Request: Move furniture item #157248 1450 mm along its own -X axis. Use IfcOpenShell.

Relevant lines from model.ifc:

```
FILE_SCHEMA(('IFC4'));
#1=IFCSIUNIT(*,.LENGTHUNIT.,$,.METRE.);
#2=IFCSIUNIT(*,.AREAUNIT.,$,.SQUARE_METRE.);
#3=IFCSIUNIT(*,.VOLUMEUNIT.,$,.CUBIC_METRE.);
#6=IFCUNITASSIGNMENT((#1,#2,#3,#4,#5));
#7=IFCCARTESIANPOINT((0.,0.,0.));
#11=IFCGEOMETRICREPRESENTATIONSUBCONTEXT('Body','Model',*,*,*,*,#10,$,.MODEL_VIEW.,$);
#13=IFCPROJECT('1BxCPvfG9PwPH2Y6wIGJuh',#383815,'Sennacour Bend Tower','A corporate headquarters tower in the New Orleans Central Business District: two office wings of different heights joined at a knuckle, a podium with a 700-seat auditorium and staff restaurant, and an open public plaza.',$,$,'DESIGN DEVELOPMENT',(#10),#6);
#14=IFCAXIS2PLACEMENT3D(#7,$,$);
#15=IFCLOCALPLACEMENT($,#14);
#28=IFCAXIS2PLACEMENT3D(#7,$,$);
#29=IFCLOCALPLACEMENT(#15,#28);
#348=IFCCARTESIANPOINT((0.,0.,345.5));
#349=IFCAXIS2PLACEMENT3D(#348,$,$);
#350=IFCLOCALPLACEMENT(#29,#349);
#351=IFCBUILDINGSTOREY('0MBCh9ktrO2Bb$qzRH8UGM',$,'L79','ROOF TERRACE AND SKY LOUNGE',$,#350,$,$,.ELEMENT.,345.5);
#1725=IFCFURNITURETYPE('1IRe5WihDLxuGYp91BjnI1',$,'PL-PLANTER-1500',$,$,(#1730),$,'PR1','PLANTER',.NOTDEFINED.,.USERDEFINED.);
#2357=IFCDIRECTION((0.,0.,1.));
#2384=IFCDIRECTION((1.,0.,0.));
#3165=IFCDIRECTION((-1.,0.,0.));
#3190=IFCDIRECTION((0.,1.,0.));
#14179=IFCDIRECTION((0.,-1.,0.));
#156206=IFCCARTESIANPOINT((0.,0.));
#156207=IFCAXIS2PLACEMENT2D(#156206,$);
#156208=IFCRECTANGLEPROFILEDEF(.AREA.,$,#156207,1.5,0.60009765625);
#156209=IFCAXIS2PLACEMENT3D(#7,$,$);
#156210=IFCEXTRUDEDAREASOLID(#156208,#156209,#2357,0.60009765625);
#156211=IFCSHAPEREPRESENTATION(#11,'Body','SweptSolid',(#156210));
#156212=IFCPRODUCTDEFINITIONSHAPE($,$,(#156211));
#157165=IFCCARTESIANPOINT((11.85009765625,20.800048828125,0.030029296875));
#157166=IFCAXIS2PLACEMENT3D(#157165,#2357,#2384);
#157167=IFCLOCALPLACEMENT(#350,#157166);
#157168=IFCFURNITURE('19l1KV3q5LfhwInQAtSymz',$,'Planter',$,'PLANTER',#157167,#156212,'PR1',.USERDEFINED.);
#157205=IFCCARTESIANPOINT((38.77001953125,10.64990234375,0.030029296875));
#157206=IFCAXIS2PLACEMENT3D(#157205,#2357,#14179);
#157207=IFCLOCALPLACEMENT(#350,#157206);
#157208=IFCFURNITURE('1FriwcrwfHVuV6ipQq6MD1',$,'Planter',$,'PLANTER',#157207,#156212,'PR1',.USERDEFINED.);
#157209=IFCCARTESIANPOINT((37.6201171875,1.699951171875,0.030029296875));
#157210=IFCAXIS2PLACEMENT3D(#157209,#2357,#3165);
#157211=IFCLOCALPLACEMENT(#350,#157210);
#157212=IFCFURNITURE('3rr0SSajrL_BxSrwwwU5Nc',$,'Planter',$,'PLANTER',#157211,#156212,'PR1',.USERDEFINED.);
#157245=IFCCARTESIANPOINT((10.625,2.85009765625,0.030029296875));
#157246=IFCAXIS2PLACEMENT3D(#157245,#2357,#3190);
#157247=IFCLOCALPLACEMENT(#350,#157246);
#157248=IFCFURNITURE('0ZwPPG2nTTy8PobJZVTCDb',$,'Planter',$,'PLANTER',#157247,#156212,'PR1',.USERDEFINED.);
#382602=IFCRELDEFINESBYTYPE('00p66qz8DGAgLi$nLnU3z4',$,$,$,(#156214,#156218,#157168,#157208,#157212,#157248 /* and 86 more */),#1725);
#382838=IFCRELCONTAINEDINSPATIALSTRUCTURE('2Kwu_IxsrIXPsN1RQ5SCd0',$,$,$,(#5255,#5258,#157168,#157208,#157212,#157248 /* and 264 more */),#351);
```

```python
import ifcopenshell
import ifcopenshell.api.geometry
import ifcopenshell.util.placement
import ifcopenshell.util.unit

model = ifcopenshell.open("model.ifc")
unit_scale = ifcopenshell.util.unit.calculate_unit_scale(model)

item = model.by_guid("0ZwPPG2nTTy8PobJZVTCDb")
matrix = ifcopenshell.util.placement.get_local_placement(item.ObjectPlacement)
matrix[:3, 3] -= matrix[:3, 0] * 1.45 / unit_scale
ifcopenshell.api.geometry.edit_object_placement(model, product=item, matrix=matrix, is_si=False)

print(ifcopenshell.util.placement.get_local_placement(item.ObjectPlacement).round(3) + 0.0)

model.write("model_rev.ifc")
```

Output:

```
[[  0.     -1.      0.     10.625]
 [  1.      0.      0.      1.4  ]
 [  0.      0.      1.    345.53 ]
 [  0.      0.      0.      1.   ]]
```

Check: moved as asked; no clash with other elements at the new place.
